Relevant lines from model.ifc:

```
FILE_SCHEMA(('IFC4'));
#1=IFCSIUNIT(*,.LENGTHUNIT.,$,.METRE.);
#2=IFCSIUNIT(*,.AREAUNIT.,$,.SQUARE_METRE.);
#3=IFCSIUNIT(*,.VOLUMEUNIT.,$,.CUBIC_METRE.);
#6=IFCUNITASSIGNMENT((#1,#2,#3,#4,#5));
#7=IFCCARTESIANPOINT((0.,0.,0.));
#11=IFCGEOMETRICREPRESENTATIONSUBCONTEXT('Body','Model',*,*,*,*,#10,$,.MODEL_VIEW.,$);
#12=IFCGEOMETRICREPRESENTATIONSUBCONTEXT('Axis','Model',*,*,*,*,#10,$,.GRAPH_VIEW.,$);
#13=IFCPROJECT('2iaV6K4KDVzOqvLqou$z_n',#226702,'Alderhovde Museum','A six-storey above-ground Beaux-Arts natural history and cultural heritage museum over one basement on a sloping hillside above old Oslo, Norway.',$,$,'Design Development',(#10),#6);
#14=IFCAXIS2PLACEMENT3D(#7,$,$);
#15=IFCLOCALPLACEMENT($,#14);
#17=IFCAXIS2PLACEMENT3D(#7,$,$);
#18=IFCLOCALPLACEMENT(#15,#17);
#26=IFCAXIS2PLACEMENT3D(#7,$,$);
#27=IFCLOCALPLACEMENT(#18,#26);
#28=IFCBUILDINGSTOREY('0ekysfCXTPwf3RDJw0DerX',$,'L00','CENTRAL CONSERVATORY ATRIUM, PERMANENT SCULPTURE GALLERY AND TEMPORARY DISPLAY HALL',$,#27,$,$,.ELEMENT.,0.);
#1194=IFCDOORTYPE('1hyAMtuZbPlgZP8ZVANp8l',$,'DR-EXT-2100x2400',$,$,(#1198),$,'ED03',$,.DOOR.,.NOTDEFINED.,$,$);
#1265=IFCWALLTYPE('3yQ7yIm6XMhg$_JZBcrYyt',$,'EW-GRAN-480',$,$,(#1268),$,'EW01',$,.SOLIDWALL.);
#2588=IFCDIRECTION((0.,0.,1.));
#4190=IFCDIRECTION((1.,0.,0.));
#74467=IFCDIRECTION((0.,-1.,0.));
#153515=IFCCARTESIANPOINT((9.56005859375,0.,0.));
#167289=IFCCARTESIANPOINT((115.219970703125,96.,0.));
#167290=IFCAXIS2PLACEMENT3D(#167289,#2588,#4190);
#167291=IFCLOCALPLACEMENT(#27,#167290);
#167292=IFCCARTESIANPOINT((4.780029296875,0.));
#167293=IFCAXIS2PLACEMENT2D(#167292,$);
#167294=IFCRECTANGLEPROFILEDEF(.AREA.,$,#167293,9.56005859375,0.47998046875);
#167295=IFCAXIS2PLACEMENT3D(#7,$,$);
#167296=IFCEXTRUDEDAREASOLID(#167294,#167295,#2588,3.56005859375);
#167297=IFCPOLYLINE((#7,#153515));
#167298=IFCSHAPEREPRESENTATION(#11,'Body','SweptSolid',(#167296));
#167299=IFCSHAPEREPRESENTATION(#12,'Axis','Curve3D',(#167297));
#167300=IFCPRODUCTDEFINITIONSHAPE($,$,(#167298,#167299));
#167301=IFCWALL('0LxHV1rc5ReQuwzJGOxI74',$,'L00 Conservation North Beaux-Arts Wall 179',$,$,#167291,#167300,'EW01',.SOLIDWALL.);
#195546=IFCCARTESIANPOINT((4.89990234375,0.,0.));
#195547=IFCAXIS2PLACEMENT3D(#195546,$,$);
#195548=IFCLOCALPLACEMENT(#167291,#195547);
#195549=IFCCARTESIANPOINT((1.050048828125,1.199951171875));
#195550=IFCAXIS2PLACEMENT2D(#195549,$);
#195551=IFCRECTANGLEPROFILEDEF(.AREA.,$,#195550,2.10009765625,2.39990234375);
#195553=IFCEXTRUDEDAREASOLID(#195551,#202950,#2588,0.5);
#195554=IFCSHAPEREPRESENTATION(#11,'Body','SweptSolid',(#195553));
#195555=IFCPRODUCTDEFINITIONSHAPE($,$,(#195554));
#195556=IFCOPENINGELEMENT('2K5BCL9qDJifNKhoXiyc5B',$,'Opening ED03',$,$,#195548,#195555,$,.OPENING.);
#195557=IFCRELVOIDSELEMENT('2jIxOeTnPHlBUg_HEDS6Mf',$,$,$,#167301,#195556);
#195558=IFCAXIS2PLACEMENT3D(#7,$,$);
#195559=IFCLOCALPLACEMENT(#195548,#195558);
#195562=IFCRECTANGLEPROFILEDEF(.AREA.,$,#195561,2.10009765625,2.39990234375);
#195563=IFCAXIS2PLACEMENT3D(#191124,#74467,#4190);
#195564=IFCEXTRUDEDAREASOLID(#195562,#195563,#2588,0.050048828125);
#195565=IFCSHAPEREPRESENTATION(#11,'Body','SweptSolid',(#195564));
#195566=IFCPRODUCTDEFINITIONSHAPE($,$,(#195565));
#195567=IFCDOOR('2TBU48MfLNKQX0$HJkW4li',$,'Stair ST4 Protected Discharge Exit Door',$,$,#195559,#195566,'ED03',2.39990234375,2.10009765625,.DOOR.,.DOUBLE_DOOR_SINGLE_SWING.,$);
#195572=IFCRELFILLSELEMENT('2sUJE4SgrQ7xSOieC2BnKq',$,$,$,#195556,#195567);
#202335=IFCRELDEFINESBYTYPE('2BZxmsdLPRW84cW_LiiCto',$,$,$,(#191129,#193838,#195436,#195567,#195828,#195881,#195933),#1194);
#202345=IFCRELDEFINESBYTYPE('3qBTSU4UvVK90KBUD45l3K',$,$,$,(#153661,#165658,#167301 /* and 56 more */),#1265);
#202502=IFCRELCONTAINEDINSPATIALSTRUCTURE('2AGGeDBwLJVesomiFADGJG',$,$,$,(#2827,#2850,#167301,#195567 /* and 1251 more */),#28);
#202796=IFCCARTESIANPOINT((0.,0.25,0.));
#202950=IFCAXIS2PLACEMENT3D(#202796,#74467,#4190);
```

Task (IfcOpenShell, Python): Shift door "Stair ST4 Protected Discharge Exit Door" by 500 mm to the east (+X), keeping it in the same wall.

```python
import ifcopenshell
import ifcopenshell.api.geometry
import ifcopenshell.util.placement
import ifcopenshell.util.unit

model = ifcopenshell.open("model.ifc")
unit_scale = ifcopenshell.util.unit.calculate_unit_scale(model)

door = model.by_id(195567)
opening = door.FillsVoids[0].RelatingOpeningElement
wall = opening.VoidsElements[0].RelatingBuildingElement

wall_matrix = ifcopenshell.util.placement.get_local_placement(wall.ObjectPlacement)
shift = wall_matrix[:3, 0] * 0.5 / unit_scale
before = ifcopenshell.util.placement.get_local_placement(door.ObjectPlacement)[:3, 3].copy()

# The door is placed relative to its opening, so it follows when the opening moves.
matrix = ifcopenshell.util.placement.get_local_placement(opening.ObjectPlacement)
matrix[:3, 3] += shift
ifcopenshell.api.geometry.edit_object_placement(
    model, product=opening, matrix=matrix, is_si=False, should_transform_children=True
)

after = ifcopenshell.util.placement.get_local_placement(door.ObjectPlacement)[:3, 3]
print("door moved by", (after - before).round(3) + 0.0)

model.write("model_rev.ifc")
```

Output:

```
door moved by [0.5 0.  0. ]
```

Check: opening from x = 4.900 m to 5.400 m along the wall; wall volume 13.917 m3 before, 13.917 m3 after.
